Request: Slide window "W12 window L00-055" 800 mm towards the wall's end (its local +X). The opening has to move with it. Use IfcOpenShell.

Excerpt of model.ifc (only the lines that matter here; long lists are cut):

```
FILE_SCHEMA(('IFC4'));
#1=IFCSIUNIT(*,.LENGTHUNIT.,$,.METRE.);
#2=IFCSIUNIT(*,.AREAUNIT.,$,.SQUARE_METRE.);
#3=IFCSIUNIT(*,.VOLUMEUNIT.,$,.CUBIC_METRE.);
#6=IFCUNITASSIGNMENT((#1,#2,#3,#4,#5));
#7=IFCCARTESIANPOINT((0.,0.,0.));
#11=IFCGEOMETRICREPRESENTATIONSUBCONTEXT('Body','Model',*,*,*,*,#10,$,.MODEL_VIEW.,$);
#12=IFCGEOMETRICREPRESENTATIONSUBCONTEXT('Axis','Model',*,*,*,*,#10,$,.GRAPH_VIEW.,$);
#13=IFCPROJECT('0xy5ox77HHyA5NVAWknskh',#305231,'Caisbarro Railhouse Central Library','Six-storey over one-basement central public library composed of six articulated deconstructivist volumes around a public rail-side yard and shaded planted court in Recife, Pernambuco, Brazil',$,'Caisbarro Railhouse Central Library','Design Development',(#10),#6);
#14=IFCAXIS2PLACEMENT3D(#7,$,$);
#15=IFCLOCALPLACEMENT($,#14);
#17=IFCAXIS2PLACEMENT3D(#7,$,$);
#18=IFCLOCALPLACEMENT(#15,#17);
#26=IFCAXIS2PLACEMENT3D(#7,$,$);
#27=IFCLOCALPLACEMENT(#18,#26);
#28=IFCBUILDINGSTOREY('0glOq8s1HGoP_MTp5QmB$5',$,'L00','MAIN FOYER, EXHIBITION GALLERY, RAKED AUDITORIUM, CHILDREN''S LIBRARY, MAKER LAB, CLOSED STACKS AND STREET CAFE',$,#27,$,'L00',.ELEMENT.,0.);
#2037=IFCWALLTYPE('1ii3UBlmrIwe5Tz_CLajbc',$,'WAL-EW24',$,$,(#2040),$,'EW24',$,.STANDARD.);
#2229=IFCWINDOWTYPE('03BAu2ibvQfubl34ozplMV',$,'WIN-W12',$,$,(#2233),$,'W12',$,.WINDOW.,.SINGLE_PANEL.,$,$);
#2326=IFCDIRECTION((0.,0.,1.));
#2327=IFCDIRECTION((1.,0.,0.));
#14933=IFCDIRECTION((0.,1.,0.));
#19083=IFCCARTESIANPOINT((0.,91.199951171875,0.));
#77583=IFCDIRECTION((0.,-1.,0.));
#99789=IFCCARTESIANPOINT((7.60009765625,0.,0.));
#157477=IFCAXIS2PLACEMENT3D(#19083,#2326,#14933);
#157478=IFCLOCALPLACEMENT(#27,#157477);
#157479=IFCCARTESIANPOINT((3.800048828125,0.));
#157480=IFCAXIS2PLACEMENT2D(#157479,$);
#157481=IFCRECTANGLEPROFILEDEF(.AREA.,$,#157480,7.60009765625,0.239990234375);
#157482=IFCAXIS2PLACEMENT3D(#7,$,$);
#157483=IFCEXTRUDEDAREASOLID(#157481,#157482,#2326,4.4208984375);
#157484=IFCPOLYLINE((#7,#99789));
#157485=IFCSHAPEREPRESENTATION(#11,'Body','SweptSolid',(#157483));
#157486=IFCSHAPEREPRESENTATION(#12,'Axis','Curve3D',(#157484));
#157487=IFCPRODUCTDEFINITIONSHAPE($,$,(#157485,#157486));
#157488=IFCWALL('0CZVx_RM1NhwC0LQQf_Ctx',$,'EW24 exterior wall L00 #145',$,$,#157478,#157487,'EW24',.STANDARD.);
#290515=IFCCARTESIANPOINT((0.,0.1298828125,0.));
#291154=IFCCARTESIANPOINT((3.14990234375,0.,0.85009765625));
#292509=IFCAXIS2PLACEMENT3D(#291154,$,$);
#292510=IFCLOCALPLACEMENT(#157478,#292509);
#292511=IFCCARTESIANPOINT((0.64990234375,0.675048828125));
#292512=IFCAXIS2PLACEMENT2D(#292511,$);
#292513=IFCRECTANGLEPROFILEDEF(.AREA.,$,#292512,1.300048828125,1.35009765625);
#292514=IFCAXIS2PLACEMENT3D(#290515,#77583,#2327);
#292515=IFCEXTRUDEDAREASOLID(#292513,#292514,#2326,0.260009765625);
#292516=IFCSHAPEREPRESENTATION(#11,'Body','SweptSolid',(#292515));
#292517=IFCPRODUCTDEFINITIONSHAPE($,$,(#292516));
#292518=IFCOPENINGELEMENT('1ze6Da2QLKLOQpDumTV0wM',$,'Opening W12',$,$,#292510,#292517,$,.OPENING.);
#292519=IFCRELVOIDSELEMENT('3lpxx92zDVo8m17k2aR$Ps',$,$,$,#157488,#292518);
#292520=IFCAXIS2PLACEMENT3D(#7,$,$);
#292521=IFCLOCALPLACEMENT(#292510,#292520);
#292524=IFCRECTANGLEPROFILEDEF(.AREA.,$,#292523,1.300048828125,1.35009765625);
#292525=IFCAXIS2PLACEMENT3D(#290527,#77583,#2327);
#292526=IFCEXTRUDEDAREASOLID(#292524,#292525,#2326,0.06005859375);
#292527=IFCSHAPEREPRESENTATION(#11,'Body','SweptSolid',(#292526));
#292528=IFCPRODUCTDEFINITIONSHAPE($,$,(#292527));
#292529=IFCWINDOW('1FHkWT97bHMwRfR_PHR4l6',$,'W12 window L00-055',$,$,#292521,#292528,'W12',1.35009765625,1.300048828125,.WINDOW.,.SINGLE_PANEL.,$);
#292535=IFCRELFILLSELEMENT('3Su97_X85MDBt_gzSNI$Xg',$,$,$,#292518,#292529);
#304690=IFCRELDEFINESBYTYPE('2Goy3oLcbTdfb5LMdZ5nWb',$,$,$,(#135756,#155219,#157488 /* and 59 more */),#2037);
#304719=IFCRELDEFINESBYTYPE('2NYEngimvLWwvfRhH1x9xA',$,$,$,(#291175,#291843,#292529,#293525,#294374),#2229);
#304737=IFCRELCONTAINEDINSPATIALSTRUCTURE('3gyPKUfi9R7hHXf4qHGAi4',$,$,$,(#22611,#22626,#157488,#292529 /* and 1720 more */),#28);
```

```python
import ifcopenshell
import ifcopenshell.api.geometry
import ifcopenshell.util.placement
import ifcopenshell.util.unit

model = ifcopenshell.open("model.ifc")
unit_scale = ifcopenshell.util.unit.calculate_unit_scale(model)

window = model.by_guid("1FHkWT97bHMwRfR_PHR4l6")
opening = window.FillsVoids[0].RelatingOpeningElement
wall = opening.VoidsElements[0].RelatingBuildingElement

wall_matrix = ifcopenshell.util.placement.get_local_placement(wall.ObjectPlacement)
shift = wall_matrix[:3, 0] * 0.8 / unit_scale
before = ifcopenshell.util.placement.get_local_placement(window.ObjectPlacement)[:3, 3].copy()

# The window is placed relative to its opening, so it follows when the opening moves.
matrix = ifcopenshell.util.placement.get_local_placement(opening.ObjectPlacement)
matrix[:3, 3] += shift
ifcopenshell.api.geometry.edit_object_placement(
    model, product=opening, matrix=matrix, is_si=False, should_transform_children=True
)

after = ifcopenshell.util.placement.get_local_placement(window.ObjectPlacement)[:3, 3]
print("window moved by", (after - before).round(3) + 0.0)

model.write("model_rev.ifc")
```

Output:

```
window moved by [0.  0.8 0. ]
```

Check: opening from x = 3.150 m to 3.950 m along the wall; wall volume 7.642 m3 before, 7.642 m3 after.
